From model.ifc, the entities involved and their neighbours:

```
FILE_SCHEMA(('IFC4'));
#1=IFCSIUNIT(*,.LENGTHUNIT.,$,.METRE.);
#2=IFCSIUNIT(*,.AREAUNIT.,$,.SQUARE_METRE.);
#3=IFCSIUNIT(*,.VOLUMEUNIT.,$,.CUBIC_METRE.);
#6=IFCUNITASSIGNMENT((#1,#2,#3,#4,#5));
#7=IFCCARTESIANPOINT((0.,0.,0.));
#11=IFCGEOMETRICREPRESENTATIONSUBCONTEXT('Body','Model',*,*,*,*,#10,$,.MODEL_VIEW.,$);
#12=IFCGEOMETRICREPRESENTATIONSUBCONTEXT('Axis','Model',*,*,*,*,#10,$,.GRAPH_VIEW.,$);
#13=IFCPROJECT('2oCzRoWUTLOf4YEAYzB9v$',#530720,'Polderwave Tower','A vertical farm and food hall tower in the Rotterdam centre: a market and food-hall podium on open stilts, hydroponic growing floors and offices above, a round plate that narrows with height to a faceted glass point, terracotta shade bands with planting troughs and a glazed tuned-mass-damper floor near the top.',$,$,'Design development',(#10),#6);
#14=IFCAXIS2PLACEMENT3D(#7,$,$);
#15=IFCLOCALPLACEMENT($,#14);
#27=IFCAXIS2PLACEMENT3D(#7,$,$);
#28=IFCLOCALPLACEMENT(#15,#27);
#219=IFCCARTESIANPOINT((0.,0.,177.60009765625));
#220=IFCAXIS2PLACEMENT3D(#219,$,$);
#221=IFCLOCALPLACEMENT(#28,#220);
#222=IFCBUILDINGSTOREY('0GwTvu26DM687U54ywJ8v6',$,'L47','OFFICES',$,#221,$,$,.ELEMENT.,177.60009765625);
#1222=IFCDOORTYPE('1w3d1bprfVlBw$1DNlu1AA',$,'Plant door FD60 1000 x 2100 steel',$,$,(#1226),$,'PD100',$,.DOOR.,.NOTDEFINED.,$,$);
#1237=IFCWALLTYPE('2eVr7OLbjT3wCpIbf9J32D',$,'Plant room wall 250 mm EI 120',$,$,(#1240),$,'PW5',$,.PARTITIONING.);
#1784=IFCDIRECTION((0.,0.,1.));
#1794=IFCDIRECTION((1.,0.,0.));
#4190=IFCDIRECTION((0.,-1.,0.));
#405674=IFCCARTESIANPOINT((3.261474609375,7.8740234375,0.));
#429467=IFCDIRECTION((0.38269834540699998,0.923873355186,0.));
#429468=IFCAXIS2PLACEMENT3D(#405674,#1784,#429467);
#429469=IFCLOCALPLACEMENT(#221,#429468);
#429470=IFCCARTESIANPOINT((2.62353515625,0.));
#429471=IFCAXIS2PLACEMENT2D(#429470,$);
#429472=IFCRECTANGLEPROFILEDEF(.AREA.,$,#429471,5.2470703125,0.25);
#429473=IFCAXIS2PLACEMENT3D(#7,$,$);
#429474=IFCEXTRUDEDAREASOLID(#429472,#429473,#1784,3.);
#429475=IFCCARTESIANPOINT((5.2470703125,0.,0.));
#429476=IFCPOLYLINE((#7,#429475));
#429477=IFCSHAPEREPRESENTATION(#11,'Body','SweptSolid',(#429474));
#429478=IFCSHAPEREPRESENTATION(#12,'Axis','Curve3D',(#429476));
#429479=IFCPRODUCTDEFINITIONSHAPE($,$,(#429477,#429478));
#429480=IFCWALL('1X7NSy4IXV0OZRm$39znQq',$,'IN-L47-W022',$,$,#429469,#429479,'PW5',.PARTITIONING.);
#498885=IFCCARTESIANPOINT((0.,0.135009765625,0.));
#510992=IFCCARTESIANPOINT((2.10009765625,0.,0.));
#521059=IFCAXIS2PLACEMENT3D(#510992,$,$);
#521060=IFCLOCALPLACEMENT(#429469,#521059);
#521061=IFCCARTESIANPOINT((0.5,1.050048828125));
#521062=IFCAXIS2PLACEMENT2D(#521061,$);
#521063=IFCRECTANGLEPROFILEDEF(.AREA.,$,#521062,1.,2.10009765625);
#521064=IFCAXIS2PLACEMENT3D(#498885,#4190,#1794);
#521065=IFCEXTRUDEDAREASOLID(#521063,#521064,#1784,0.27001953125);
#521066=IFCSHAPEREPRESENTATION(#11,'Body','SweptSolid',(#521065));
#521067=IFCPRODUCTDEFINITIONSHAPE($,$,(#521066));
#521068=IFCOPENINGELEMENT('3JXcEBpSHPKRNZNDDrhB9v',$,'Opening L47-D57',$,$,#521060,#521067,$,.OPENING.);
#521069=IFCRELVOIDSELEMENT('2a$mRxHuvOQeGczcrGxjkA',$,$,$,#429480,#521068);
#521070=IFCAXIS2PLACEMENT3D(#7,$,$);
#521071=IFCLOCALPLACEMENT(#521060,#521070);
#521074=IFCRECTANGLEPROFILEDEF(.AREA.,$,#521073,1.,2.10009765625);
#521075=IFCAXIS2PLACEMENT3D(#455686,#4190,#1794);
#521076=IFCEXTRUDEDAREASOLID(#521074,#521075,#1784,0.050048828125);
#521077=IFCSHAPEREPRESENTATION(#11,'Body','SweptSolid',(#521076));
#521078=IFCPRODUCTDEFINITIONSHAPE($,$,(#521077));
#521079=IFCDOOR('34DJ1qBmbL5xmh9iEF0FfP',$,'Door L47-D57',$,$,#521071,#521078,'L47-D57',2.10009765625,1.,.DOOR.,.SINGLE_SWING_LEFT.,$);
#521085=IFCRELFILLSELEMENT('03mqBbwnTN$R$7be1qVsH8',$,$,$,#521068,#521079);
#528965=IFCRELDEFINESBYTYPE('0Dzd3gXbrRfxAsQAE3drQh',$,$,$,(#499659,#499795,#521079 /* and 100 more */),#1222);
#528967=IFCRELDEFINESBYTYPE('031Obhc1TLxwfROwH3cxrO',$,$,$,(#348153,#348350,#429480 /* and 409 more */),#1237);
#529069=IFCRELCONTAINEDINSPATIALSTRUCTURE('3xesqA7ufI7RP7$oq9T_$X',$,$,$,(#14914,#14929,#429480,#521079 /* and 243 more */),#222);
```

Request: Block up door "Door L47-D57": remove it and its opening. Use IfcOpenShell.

```python
import ifcopenshell
import ifcopenshell.api.feature
import ifcopenshell.api.root
import ifcopenshell.geom
import ifcopenshell.util.shape

model = ifcopenshell.open("model.ifc")
settings = ifcopenshell.geom.settings()


def volume(element):
    """Net volume in cubic metres, openings subtracted."""
    shape = ifcopenshell.geom.create_shape(settings, element)
    return ifcopenshell.util.shape.get_volume(shape.geometry)


door = model.by_guid("34DJ1qBmbL5xmh9iEF0FfP")
opening = door.FillsVoids[0].RelatingOpeningElement
wall = opening.VoidsElements[0].RelatingBuildingElement
before = volume(wall)

ifcopenshell.api.root.remove_product(model, product=door)
ifcopenshell.api.feature.remove_feature(model, feature=opening)

after = volume(wall)

print(f"wall volume {before:.3f} -> {after:.3f} m3")

model.write("model_edited.ifc")
```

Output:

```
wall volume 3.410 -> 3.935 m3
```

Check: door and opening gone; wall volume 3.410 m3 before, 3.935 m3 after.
